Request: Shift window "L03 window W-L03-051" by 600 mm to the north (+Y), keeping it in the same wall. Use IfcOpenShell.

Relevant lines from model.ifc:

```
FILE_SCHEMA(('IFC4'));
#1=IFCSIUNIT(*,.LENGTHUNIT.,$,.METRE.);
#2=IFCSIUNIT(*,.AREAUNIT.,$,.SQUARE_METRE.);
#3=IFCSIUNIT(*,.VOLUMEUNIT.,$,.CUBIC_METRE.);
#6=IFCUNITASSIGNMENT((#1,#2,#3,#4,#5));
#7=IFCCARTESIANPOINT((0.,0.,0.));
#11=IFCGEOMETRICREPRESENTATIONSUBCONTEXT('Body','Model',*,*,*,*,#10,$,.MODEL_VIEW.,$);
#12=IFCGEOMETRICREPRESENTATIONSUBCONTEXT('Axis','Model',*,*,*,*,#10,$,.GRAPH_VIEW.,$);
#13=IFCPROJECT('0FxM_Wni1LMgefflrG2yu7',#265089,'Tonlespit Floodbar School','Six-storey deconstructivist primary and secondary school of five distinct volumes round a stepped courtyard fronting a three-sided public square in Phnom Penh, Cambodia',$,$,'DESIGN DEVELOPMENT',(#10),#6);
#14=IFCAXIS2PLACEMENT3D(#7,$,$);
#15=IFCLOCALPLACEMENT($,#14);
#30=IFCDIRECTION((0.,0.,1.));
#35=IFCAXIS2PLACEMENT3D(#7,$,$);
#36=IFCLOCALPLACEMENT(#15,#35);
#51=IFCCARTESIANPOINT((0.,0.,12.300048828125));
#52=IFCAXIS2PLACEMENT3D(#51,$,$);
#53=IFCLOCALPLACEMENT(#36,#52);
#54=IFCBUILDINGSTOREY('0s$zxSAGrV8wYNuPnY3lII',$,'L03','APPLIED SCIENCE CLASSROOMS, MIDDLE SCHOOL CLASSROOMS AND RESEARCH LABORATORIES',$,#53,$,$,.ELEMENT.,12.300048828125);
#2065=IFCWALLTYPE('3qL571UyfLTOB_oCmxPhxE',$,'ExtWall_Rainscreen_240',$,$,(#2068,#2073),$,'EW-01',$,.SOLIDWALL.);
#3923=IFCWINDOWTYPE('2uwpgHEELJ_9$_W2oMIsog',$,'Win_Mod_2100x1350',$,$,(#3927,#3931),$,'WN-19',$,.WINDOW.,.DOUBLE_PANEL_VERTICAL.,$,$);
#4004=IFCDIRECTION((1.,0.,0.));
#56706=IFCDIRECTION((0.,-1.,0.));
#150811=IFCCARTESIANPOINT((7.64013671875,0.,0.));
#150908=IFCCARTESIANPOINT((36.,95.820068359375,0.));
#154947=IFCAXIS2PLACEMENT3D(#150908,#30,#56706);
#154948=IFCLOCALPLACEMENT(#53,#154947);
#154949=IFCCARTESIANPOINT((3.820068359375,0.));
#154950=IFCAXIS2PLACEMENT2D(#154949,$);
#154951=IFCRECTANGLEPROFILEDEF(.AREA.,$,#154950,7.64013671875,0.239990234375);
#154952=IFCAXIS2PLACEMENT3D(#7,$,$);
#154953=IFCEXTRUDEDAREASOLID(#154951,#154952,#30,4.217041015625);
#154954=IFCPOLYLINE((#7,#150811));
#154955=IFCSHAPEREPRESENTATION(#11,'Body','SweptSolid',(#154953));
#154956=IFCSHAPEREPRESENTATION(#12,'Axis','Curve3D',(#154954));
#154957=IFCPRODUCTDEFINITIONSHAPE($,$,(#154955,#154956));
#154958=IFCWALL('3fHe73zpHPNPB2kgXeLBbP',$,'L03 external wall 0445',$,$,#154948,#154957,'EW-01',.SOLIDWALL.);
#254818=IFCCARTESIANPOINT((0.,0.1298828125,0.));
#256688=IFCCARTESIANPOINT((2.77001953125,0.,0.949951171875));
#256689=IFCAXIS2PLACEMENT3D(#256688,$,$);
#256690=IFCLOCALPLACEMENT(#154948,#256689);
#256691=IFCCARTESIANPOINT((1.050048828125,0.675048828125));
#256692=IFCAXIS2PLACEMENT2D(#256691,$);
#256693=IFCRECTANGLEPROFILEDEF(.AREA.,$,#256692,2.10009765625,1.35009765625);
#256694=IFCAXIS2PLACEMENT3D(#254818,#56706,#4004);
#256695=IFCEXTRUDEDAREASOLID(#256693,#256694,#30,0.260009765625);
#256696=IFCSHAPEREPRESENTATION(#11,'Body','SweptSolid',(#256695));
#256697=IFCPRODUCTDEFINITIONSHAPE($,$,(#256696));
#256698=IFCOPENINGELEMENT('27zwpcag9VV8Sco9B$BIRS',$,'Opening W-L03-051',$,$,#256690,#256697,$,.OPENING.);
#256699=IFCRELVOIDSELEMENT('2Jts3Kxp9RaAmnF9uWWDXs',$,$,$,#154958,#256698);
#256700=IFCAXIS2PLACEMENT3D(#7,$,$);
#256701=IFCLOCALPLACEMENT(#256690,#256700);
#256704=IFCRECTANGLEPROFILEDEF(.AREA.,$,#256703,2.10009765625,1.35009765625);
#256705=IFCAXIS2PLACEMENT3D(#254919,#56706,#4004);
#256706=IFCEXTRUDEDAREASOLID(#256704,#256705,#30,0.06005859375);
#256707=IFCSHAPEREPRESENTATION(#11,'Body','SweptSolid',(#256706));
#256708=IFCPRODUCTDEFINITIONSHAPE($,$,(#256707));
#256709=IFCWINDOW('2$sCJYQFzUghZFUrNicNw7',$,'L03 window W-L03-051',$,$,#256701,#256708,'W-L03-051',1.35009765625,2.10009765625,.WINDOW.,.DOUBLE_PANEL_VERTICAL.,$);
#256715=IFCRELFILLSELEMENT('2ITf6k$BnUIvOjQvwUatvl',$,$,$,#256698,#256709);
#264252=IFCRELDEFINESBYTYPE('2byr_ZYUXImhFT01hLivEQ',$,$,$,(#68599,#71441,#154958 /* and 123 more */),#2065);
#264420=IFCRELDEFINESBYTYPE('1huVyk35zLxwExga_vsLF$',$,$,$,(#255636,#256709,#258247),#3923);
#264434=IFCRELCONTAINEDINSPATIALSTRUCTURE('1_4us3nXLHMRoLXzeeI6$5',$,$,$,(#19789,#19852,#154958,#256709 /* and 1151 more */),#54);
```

```python
import ifcopenshell
import ifcopenshell.api.geometry
import ifcopenshell.util.placement
import ifcopenshell.util.unit

model = ifcopenshell.open("model.ifc")
unit_scale = ifcopenshell.util.unit.calculate_unit_scale(model)

window = model.by_id(256709)
opening = window.FillsVoids[0].RelatingOpeningElement
wall = opening.VoidsElements[0].RelatingBuildingElement

wall_matrix = ifcopenshell.util.placement.get_local_placement(wall.ObjectPlacement)
shift = wall_matrix[:3, 0] * -0.6 / unit_scale
before = ifcopenshell.util.placement.get_local_placement(window.ObjectPlacement)[:3, 3].copy()

# The window is placed relative to its opening, so it follows when the opening moves.
matrix = ifcopenshell.util.placement.get_local_placement(opening.ObjectPlacement)
matrix[:3, 3] += shift
ifcopenshell.api.geometry.edit_object_placement(
    model, product=opening, matrix=matrix, is_si=False, should_transform_children=True
)

after = ifcopenshell.util.placement.get_local_placement(window.ObjectPlacement)[:3, 3]
print("window moved by", (after - before).round(3) + 0.0)

model.write("model_v2.ifc")
```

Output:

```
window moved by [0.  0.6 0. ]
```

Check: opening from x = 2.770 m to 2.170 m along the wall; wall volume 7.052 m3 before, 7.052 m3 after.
